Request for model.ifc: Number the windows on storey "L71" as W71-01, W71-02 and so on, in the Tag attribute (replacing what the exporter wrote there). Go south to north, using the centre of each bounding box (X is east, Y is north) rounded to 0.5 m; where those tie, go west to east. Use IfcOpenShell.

First a look at what the model holds.

```python
import ifcopenshell
import ifcopenshell.util.element
import ifcopenshell.util.placement

model = ifcopenshell.open("model.ifc")
print(model.schema)
storey = next(s for s in model.by_type("IfcBuildingStorey") if s.Name == "L71")
windows = [e for e in ifcopenshell.util.element.get_decomposition(storey) if e.is_a("IfcWindow")]
for e in sorted(windows, key=lambda e: e.id()):
    origin = ifcopenshell.util.placement.get_local_placement(e.ObjectPlacement)[:3, 3]
    print(e.id(), e.Tag, e.Name, origin.round(2) + 0.0, sep=" | ")
```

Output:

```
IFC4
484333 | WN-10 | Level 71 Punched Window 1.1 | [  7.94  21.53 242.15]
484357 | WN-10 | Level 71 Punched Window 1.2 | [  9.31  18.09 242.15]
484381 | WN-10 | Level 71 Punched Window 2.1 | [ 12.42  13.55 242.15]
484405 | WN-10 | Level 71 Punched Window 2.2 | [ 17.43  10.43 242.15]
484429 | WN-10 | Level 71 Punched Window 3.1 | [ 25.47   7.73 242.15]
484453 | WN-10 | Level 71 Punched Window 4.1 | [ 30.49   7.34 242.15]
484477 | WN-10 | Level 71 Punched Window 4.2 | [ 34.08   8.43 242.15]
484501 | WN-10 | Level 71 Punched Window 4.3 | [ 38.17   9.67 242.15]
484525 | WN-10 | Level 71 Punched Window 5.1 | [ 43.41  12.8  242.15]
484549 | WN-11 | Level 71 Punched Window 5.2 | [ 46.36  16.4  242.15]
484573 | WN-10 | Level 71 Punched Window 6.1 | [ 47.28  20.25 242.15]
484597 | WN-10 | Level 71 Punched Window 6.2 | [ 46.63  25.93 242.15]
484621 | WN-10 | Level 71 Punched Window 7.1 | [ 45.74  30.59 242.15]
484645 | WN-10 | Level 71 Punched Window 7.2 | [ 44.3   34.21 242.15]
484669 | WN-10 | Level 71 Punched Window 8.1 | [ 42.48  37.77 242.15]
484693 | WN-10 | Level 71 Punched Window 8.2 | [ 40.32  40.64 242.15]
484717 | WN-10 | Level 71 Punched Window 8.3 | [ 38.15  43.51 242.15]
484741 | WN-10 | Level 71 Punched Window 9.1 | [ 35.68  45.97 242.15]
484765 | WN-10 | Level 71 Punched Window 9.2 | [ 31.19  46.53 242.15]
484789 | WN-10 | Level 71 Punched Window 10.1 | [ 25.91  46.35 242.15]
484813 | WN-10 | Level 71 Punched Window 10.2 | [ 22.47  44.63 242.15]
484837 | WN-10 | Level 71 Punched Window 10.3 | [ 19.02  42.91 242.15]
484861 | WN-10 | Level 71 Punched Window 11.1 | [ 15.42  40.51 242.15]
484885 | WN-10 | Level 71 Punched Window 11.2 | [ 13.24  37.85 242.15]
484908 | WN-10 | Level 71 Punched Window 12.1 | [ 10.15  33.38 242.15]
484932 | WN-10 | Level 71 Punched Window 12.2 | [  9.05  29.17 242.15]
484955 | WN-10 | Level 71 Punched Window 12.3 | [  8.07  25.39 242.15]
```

```python
import ifcopenshell
import ifcopenshell.geom
import ifcopenshell.util.element
import ifcopenshell.util.shape

model = ifcopenshell.open("model.ifc")
settings = ifcopenshell.geom.settings()
settings.set("use-world-coords", True)


def centre(element):
    shape = ifcopenshell.geom.create_shape(settings, element)
    return ifcopenshell.util.shape.get_bbox_centroid(shape.geometry)


storey = next(s for s in model.by_type("IfcBuildingStorey") if s.Name == "L71")
windows = [e for e in ifcopenshell.util.element.get_decomposition(storey) if e.is_a("IfcWindow")]

# Insertion points can sit at a corner or the storey origin, so sort by the geometry (in metres).
centres = {e: centre(e) for e in windows}
windows.sort(key=lambda e: (round(centres[e][1] / 0.5), centres[e][0]))

for i, e in enumerate(windows, start=1):
    number = f"W71-{i:02d}"
    e.Tag = number
    print(e.id(), number)

model.write("model_rev.ifc")
```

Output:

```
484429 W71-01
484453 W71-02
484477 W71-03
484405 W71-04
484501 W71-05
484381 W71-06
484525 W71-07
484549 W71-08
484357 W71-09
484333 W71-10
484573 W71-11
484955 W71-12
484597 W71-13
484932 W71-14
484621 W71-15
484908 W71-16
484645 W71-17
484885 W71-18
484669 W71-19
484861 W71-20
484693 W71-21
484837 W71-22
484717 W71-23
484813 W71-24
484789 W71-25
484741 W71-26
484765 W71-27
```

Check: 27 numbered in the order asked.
